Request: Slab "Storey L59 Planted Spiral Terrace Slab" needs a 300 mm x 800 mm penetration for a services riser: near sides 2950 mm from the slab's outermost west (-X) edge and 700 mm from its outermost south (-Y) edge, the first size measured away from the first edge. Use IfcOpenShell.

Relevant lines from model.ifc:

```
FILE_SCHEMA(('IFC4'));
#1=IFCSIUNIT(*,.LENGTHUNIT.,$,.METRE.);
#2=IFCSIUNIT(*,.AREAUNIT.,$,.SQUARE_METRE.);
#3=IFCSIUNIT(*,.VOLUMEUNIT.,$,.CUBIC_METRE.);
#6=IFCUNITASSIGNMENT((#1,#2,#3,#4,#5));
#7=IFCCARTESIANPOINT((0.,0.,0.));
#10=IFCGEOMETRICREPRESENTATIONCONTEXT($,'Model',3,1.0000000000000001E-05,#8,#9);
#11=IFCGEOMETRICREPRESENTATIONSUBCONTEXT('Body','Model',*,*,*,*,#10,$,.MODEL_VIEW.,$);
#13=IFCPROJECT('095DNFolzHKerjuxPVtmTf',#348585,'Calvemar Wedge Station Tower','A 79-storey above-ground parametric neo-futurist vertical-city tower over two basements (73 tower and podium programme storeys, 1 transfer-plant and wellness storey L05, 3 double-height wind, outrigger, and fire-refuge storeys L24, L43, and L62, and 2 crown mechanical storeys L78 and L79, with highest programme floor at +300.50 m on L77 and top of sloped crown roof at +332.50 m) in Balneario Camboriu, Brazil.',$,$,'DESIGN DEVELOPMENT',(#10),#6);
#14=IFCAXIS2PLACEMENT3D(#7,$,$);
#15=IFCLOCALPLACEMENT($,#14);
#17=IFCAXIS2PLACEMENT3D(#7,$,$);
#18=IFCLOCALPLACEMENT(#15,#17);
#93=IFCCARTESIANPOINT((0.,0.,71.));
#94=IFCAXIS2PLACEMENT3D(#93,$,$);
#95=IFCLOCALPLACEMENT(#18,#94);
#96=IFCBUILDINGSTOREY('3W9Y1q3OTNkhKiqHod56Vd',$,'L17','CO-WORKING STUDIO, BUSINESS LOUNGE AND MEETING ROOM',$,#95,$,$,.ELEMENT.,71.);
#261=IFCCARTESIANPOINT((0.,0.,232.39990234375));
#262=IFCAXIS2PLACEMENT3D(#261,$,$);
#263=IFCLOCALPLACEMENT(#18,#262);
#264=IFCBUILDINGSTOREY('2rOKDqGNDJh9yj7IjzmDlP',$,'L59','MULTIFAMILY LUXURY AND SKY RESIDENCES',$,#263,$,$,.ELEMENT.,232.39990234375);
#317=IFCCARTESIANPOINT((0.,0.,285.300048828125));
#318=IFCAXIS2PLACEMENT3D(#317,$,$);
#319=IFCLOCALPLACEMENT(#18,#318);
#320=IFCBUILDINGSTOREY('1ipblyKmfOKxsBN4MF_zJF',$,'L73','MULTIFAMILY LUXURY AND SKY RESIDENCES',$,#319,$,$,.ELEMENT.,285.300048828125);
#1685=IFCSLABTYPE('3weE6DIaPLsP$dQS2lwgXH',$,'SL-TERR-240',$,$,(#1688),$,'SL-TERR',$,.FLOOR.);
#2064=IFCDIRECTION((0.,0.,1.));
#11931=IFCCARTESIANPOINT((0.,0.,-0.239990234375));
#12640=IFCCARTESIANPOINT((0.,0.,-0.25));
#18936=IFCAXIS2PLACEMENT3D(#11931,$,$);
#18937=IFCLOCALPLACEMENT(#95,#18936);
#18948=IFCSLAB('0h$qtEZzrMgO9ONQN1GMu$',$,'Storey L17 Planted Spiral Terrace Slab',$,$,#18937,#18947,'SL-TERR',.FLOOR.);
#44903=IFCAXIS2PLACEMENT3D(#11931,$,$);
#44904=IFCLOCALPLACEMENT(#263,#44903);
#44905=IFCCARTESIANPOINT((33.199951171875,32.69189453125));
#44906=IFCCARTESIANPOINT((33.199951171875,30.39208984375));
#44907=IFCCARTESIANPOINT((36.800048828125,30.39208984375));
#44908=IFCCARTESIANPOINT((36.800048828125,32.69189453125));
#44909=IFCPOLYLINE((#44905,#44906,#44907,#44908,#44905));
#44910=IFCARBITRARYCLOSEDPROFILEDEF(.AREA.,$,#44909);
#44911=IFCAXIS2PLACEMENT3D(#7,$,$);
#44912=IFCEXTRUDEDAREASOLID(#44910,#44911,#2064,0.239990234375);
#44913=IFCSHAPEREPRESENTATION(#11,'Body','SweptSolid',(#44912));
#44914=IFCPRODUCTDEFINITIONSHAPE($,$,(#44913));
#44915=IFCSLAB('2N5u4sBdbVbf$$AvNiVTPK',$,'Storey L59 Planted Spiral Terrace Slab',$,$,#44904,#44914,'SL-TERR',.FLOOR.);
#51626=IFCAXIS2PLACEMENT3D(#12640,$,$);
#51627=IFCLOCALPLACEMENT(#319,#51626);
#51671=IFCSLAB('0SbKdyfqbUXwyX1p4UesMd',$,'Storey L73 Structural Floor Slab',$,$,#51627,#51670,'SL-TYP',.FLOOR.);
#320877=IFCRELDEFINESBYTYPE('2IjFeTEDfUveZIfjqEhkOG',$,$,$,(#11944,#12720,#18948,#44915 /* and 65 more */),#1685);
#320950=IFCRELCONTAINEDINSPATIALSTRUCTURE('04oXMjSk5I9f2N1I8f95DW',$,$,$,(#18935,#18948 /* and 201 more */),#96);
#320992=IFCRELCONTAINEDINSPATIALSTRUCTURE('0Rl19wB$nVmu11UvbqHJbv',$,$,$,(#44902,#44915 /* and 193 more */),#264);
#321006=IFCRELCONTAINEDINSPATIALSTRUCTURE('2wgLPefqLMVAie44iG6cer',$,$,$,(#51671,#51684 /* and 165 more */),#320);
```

```python
import numpy as np
import ifcopenshell
import ifcopenshell.api.feature
import ifcopenshell.api.geometry
import ifcopenshell.api.root
import ifcopenshell.geom
import ifcopenshell.util.placement
import ifcopenshell.util.representation
import ifcopenshell.util.shape
import ifcopenshell.util.unit

model = ifcopenshell.open("model.ifc")
unit_scale = ifcopenshell.util.unit.calculate_unit_scale(model)
settings = ifcopenshell.geom.settings()


def volume(element):
    """Net volume in cubic metres, openings subtracted."""
    shape = ifcopenshell.geom.create_shape(settings, element)
    return ifcopenshell.util.shape.get_volume(shape.geometry)


slab = model.by_guid("2N5u4sBdbVbf$$AvNiVTPK")
before = volume(slab)

# Extent in the slab's own axes, in metres. The edges named are its -X and -Y sides.
slab_shape = ifcopenshell.geom.create_shape(settings, slab)
vertices = ifcopenshell.util.shape.get_vertices(slab_shape.geometry)
x_min, y_min, bottom = vertices.min(axis=0)
top = vertices[:, 2].max()

opening = ifcopenshell.api.root.create_entity(model, ifc_class="IfcOpeningElement", name="Services riser opening", predefined_type="OPENING")
context = ifcopenshell.util.representation.get_context(model, "Model", "Body", "MODEL_VIEW")
width, depth = 0.3, 0.8
outline = [(0.0, 0.0), (width, 0.0), (width, depth), (0.0, depth), (0.0, 0.0)]
# Overshoot both faces by 50 mm so the cut is clean.
shape = ifcopenshell.api.geometry.add_slab_representation(
    model, context=context, depth=top - bottom + 0.1, polyline=outline
)
ifcopenshell.api.geometry.assign_representation(model, product=opening, representation=shape)

matrix = ifcopenshell.util.placement.get_local_placement(slab.ObjectPlacement)
matrix[:, 3] = matrix @ np.append(np.array([x_min + 2.95, y_min + 0.7, bottom - 0.05]) / unit_scale, 1.0)
ifcopenshell.api.geometry.edit_object_placement(model, product=opening, matrix=matrix, is_si=False)
ifcopenshell.api.feature.add_feature(model, feature=opening, element=slab)

after = volume(slab)

print(f"slab volume {before:.3f} -> {after:.3f} m3")

model.write("model_v2.ifc")
```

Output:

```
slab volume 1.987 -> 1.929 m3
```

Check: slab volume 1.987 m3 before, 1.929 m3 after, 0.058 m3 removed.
